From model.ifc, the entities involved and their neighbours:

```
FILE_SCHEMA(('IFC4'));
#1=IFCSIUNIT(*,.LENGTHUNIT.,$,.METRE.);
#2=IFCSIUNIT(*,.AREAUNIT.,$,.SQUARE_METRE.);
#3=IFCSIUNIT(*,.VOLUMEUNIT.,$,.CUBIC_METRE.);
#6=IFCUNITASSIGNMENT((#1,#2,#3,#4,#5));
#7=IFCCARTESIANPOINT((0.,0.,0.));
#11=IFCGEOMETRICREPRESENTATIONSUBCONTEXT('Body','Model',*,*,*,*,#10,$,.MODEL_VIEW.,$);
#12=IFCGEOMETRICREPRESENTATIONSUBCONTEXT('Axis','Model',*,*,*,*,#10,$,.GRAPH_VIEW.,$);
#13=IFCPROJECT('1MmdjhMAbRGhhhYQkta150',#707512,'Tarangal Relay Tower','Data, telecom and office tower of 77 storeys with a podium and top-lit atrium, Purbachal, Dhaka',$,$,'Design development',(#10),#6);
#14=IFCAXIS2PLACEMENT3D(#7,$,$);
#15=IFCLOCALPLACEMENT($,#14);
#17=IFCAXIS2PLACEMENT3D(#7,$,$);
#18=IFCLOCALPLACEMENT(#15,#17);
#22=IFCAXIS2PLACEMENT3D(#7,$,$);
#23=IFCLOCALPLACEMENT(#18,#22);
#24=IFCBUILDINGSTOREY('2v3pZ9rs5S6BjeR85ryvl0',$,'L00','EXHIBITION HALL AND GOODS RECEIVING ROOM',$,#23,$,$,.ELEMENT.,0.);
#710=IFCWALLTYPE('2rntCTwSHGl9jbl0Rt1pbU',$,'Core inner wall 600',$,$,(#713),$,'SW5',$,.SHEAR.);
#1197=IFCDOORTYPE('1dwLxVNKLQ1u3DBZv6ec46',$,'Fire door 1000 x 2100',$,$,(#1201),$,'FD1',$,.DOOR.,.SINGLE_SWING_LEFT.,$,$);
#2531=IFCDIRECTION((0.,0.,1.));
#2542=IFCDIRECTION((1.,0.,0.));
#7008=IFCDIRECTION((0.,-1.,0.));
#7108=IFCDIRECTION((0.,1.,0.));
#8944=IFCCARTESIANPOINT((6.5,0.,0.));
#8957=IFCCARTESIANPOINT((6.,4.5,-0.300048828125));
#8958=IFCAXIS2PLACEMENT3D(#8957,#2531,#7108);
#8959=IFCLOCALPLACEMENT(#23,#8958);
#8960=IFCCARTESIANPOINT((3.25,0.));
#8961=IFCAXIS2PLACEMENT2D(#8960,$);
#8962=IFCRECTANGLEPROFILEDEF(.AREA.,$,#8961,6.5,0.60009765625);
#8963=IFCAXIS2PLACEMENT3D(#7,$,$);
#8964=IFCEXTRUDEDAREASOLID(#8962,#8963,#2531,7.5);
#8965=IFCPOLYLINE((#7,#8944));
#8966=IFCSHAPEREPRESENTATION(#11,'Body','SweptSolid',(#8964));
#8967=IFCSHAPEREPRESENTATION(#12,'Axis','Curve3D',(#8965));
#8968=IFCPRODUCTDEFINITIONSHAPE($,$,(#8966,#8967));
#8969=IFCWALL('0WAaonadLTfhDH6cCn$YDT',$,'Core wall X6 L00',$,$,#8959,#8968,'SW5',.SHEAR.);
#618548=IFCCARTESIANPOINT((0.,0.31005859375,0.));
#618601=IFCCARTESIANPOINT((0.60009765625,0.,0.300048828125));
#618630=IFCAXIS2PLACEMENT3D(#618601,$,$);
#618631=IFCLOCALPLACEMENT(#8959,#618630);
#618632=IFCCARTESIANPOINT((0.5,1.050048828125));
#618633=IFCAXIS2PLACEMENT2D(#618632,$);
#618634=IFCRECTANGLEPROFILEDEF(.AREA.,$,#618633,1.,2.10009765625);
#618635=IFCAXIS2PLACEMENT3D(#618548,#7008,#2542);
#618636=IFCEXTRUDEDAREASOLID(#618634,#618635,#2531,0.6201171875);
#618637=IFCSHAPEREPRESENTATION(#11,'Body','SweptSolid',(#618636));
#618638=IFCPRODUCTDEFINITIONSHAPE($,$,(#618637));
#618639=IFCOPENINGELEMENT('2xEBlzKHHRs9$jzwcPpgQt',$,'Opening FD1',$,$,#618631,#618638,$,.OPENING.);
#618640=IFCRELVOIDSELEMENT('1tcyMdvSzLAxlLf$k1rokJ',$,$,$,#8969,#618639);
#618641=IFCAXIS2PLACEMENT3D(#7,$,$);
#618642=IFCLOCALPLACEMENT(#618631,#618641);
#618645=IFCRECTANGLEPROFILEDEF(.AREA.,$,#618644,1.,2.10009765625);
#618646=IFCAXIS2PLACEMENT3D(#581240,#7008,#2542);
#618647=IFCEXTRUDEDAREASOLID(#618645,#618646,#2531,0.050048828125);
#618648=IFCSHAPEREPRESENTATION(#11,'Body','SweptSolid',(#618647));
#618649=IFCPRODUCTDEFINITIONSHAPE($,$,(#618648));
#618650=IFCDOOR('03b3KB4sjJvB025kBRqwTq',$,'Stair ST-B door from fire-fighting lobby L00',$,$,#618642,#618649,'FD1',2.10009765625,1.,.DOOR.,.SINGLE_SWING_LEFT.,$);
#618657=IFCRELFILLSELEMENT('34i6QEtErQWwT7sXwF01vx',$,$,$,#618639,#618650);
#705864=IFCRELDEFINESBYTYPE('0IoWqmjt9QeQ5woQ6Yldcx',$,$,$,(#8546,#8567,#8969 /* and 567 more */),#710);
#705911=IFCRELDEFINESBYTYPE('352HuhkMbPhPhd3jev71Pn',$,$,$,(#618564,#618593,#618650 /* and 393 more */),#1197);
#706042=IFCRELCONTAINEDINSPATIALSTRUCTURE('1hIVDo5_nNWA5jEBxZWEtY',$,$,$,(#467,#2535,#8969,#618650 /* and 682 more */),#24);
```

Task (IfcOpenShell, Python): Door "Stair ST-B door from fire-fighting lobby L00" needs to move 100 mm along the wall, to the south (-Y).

```python
import ifcopenshell
import ifcopenshell.api.geometry
import ifcopenshell.util.placement

model = ifcopenshell.open("model.ifc")

door = model.by_guid("03b3KB4sjJvB025kBRqwTq")
opening = door.FillsVoids[0].RelatingOpeningElement
wall = opening.VoidsElements[0].RelatingBuildingElement

wall_matrix = ifcopenshell.util.placement.get_local_placement(wall.ObjectPlacement)
shift = wall_matrix[:3, 0] * -0.1
before = ifcopenshell.util.placement.get_local_placement(door.ObjectPlacement)[:3, 3].copy()

# The door is placed relative to its opening, so it follows when the opening moves.
matrix = ifcopenshell.util.placement.get_local_placement(opening.ObjectPlacement)
matrix[:3, 3] += shift
ifcopenshell.api.geometry.edit_object_placement(
    model, product=opening, matrix=matrix, is_si=False, should_transform_children=True
)

after = ifcopenshell.util.placement.get_local_placement(door.ObjectPlacement)[:3, 3]
print("door moved by", (after - before).round(3) + 0.0)

model.write("model_updated.ifc")
```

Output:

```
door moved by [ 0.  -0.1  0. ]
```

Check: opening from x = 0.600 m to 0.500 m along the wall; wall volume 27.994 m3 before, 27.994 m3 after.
